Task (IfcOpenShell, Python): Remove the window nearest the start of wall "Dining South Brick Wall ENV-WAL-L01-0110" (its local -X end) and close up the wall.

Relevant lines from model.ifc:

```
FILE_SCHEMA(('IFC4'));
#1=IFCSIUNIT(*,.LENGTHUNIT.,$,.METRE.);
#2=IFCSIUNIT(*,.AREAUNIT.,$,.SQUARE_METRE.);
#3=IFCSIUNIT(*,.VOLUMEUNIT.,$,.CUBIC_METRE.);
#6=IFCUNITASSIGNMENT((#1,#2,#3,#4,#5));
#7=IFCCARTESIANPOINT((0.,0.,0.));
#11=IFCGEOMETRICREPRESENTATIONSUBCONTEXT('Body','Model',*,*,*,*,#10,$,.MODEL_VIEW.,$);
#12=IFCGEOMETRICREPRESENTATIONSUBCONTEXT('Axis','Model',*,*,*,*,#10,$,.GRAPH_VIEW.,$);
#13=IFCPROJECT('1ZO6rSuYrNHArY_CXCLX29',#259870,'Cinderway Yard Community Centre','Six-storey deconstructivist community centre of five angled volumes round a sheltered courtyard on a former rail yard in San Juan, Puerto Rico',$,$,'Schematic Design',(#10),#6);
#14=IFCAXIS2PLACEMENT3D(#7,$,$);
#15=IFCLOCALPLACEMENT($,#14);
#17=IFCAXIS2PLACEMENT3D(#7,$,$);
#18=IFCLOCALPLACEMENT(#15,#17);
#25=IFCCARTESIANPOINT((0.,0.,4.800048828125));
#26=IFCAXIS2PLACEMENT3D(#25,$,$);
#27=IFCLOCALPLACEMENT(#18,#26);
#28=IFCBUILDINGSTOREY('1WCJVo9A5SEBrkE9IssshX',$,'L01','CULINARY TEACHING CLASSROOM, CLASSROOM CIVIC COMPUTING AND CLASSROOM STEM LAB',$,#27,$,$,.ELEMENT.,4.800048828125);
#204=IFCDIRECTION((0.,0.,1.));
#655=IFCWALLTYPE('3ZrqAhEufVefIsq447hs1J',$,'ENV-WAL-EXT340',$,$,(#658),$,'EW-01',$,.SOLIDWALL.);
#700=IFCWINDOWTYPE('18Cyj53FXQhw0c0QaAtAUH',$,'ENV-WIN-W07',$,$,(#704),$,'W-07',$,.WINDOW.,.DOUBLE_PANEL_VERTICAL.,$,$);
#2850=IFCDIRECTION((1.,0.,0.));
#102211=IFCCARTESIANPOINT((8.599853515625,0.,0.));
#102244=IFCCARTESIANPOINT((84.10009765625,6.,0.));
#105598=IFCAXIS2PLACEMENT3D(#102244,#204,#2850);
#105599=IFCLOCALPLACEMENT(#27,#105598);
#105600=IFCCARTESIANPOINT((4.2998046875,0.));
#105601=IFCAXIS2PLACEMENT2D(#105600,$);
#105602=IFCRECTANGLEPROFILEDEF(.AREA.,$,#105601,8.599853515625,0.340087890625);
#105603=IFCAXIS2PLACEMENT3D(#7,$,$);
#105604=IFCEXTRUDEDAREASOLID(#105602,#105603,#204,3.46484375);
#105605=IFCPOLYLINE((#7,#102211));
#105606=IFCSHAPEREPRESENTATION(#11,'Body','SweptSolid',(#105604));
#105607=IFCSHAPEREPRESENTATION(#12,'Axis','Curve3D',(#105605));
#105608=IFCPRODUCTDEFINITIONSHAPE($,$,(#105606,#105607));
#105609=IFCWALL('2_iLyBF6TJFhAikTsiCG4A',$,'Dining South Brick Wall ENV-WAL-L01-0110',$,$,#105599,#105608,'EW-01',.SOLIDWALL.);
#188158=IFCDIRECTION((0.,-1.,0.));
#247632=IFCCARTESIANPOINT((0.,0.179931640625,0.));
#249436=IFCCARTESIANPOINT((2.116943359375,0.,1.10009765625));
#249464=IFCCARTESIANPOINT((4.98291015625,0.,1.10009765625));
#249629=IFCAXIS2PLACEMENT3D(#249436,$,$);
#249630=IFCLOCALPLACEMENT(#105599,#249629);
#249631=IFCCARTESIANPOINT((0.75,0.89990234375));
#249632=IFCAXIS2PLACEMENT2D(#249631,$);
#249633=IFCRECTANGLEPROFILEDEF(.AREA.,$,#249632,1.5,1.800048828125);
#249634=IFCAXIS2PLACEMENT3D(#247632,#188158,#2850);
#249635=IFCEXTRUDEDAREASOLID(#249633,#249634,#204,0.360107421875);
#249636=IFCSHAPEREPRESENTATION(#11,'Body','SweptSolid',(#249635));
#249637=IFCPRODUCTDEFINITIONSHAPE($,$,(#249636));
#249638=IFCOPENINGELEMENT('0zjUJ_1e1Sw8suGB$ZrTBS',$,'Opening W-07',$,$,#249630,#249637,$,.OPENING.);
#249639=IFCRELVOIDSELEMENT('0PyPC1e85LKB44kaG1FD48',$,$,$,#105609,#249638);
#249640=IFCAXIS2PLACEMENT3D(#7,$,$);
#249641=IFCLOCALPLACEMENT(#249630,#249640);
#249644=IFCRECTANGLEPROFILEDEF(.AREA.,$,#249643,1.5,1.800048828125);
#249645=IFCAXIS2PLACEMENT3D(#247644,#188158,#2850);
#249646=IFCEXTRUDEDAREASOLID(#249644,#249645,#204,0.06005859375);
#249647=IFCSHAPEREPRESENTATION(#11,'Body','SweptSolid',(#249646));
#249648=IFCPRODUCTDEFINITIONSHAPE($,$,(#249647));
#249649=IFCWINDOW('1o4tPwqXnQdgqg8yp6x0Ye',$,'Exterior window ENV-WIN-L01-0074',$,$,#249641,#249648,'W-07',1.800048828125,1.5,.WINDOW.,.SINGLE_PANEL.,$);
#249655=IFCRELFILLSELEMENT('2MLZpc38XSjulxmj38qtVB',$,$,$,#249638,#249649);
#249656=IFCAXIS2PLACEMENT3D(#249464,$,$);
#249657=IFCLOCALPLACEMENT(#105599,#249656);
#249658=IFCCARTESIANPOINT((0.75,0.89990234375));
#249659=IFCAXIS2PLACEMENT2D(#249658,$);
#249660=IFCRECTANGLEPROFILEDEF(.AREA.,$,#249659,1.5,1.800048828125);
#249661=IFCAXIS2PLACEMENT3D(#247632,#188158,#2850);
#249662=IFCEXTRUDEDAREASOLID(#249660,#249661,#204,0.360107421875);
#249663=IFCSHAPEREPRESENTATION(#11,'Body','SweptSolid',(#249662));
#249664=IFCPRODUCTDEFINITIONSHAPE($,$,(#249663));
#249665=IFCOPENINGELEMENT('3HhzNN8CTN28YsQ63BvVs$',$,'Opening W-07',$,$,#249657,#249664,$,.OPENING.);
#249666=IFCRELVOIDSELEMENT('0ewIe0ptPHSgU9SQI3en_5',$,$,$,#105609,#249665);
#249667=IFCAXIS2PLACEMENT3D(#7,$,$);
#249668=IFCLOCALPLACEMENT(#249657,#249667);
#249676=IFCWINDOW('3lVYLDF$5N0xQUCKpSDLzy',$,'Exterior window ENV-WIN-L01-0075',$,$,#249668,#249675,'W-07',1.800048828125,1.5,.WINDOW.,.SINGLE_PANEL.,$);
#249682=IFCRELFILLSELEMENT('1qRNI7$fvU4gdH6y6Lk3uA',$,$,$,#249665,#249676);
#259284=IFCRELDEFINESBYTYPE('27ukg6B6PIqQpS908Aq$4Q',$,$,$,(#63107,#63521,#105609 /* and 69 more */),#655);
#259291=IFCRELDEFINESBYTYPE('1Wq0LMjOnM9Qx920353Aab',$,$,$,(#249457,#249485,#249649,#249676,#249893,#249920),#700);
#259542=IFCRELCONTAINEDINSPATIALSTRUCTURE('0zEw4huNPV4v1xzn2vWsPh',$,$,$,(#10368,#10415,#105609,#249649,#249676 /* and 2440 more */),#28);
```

```python
import ifcopenshell
import ifcopenshell.api.feature
import ifcopenshell.api.root
import ifcopenshell.geom
import ifcopenshell.util.shape

model = ifcopenshell.open("model.ifc")
settings = ifcopenshell.geom.settings()


def volume(element):
    """Net volume in cubic metres, openings subtracted."""
    shape = ifcopenshell.geom.create_shape(settings, element)
    return ifcopenshell.util.shape.get_volume(shape.geometry)


window = model.by_guid("1o4tPwqXnQdgqg8yp6x0Ye")
opening = window.FillsVoids[0].RelatingOpeningElement
wall = opening.VoidsElements[0].RelatingBuildingElement
before = volume(wall)

ifcopenshell.api.root.remove_product(model, product=window)
ifcopenshell.api.feature.remove_feature(model, feature=opening)

after = volume(wall)

print(f"wall volume {before:.3f} -> {after:.3f} m3")

model.write("model_updated.ifc")
```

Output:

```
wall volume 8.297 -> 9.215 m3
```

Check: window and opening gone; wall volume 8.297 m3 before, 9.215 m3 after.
